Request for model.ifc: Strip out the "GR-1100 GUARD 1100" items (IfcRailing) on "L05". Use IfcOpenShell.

First a look at what the model holds.

```python
import ifcopenshell
import ifcopenshell.util.element

model = ifcopenshell.open("model.ifc")
print(model.schema)
storey = next(s for s in model.by_type("IfcBuildingStorey") if s.Name == "L05")
railings = [e for e in ifcopenshell.util.element.get_decomposition(storey) if e.is_a("IfcRailing")]
seen = {}
for e in railings:
    element_type = ifcopenshell.util.element.get_type(e)
    name = element_type.Name if element_type not in (None, e) else None
    seen[name] = seen.get(name, 0) + 1
for name, count in sorted(seen.items(), key=str):
    print(count, "x", name)
```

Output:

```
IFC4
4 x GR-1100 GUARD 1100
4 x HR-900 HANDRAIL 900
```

```python
import ifcopenshell
import ifcopenshell.api.root
import ifcopenshell.util.element

model = ifcopenshell.open("model.ifc")

storey = next(s for s in model.by_type("IfcBuildingStorey") if s.Name == "L05")
railings = [e for e in ifcopenshell.util.element.get_decomposition(storey) if e.is_a("IfcRailing")]
targets = [e for e in railings if (t := ifcopenshell.util.element.get_type(e)) not in (None, e) and t.Name == "GR-1100 GUARD 1100"]

for e in targets:
    ifcopenshell.api.root.remove_product(model, product=e)
print(len(targets), "removed")

model.write("model_updated.ifc")
```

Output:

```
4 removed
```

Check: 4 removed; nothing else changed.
